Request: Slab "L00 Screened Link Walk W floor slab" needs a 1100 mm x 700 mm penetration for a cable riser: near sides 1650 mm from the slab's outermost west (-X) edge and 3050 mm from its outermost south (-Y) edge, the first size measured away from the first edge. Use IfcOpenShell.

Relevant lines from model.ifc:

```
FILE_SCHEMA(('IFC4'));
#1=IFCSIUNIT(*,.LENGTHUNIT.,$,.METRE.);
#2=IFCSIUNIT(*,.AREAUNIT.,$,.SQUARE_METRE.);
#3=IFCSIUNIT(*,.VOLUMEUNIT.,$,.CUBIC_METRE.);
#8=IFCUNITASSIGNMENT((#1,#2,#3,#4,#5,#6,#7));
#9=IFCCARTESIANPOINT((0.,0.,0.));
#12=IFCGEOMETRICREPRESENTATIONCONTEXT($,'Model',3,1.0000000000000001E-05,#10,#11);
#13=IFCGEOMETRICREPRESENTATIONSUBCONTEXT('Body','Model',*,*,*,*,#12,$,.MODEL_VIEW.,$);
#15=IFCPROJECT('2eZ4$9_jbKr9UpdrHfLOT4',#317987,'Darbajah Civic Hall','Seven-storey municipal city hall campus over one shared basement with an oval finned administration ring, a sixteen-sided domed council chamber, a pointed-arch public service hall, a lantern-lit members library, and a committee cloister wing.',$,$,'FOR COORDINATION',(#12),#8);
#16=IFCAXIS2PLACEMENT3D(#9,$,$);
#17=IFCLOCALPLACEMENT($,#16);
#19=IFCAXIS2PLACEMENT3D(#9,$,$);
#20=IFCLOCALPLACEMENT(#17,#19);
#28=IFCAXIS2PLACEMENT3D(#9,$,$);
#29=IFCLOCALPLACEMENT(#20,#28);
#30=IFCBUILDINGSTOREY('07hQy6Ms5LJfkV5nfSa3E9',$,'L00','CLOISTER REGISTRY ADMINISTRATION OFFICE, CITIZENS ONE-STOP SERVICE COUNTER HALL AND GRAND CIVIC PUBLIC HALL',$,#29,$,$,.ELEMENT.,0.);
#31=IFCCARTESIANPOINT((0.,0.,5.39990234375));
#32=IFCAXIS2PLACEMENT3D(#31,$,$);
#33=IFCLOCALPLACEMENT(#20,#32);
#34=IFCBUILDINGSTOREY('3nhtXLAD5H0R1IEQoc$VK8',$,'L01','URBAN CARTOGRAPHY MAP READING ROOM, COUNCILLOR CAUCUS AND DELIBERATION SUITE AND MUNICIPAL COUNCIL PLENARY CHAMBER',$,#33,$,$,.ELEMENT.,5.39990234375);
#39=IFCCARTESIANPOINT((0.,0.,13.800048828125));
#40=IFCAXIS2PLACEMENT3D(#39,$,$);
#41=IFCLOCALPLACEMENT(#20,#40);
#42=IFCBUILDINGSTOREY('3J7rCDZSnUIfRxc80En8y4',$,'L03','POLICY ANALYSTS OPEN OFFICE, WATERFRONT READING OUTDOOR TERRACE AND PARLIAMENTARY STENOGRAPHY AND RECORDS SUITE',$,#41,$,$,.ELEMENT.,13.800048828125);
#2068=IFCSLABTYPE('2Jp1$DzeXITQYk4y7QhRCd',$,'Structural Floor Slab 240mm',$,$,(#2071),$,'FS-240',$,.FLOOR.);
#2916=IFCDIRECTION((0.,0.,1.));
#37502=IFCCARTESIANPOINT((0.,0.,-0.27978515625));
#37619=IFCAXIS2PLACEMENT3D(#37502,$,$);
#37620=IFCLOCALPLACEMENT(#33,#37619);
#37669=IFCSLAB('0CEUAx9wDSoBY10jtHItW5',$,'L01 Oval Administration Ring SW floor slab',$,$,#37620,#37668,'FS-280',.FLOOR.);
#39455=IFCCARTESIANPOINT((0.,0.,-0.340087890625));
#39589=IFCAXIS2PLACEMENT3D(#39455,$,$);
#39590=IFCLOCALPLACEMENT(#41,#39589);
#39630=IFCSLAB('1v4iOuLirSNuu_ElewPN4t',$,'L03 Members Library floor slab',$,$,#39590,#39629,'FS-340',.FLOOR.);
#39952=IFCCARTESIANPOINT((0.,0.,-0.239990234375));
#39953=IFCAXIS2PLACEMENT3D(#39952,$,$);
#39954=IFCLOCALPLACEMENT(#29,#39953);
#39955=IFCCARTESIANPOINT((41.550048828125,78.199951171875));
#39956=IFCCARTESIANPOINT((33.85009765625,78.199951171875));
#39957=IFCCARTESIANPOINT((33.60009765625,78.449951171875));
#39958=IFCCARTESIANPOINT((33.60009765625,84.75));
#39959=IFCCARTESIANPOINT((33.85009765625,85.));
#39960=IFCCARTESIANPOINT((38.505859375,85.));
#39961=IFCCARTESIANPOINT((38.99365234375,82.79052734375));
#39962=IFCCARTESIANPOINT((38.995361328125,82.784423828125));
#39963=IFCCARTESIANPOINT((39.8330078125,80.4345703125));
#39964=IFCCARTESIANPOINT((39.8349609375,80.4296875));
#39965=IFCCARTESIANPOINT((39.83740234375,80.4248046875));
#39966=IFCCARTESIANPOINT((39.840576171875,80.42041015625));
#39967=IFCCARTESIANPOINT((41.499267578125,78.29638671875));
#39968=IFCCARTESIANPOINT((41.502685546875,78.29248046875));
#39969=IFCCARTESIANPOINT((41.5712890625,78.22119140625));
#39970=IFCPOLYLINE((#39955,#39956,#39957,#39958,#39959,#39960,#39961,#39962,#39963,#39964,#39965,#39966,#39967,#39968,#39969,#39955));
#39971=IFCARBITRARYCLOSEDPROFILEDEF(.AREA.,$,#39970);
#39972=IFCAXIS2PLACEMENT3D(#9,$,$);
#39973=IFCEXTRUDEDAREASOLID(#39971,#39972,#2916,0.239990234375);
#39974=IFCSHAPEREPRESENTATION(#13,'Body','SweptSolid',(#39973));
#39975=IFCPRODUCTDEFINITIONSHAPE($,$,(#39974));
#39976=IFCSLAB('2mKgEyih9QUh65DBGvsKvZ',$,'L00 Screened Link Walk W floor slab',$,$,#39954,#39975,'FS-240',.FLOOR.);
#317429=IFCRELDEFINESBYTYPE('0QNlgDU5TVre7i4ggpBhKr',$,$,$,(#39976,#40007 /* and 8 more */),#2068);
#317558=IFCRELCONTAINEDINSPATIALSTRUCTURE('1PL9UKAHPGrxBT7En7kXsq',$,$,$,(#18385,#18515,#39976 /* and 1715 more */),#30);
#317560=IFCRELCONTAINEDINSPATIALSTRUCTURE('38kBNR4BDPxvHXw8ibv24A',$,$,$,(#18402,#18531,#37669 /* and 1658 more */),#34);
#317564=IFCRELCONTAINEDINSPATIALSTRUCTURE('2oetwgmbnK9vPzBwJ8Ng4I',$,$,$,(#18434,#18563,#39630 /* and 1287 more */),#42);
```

```python
import numpy as np
import ifcopenshell
import ifcopenshell.api.feature
import ifcopenshell.api.geometry
import ifcopenshell.api.root
import ifcopenshell.geom
import ifcopenshell.util.placement
import ifcopenshell.util.representation
import ifcopenshell.util.shape
import ifcopenshell.util.unit

model = ifcopenshell.open("model.ifc")
unit_scale = ifcopenshell.util.unit.calculate_unit_scale(model)
settings = ifcopenshell.geom.settings()


def volume(element):
    """Net volume in cubic metres, openings subtracted."""
    shape = ifcopenshell.geom.create_shape(settings, element)
    return ifcopenshell.util.shape.get_volume(shape.geometry)


slab = model.by_id(39976)
before = volume(slab)

# Extent in the slab's own axes, in metres. The edges named are its -X and -Y sides.
slab_shape = ifcopenshell.geom.create_shape(settings, slab)
vertices = ifcopenshell.util.shape.get_vertices(slab_shape.geometry)
x_min, y_min, bottom = vertices.min(axis=0)
top = vertices[:, 2].max()

opening = ifcopenshell.api.root.create_entity(model, ifc_class="IfcOpeningElement", name="Cable riser opening", predefined_type="OPENING")
context = ifcopenshell.util.representation.get_context(model, "Model", "Body", "MODEL_VIEW")
width, depth = 1.1, 0.7
outline = [(0.0, 0.0), (width, 0.0), (width, depth), (0.0, depth), (0.0, 0.0)]
# Overshoot both faces by 50 mm so the cut is clean.
shape = ifcopenshell.api.geometry.add_slab_representation(
    model, context=context, depth=top - bottom + 0.1, polyline=outline
)
ifcopenshell.api.geometry.assign_representation(model, product=opening, representation=shape)

matrix = ifcopenshell.util.placement.get_local_placement(slab.ObjectPlacement)
matrix[:, 3] = matrix @ np.append(np.array([x_min + 1.65, y_min + 3.05, bottom - 0.05]) / unit_scale, 1.0)
ifcopenshell.api.geometry.edit_object_placement(model, product=opening, matrix=matrix, is_si=False)
ifcopenshell.api.feature.add_feature(model, feature=opening, element=slab)

after = volume(slab)

print(f"slab volume {before:.3f} -> {after:.3f} m3")

model.write("model_rev.ifc")
```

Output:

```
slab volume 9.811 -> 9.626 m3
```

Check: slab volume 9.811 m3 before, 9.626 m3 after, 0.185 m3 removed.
